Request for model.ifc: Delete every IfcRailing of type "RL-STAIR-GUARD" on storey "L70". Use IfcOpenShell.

First a look at what the model holds.

```python
import ifcopenshell
import ifcopenshell.util.element

model = ifcopenshell.open("model.ifc")
print(model.schema)
storey = next(s for s in model.by_type("IfcBuildingStorey") if s.Name == "L70")
railings = [e for e in ifcopenshell.util.element.get_decomposition(storey) if e.is_a("IfcRailing")]
seen = {}
for e in railings:
    element_type = ifcopenshell.util.element.get_type(e)
    name = element_type.Name if element_type not in (None, e) else None
    seen[name] = seen.get(name, 0) + 1
for name, count in sorted(seen.items(), key=str):
    print(count, "x", name)
```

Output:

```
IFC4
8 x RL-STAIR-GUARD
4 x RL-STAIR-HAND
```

```python
import ifcopenshell
import ifcopenshell.api.root
import ifcopenshell.util.element

model = ifcopenshell.open("model.ifc")

storey = next(s for s in model.by_type("IfcBuildingStorey") if s.Name == "L70")
railings = [e for e in ifcopenshell.util.element.get_decomposition(storey) if e.is_a("IfcRailing")]
targets = [e for e in railings if (t := ifcopenshell.util.element.get_type(e)) not in (None, e) and t.Name == "RL-STAIR-GUARD"]

for e in targets:
    ifcopenshell.api.root.remove_product(model, product=e)
print(len(targets), "removed")

model.write("model_edited.ifc")
```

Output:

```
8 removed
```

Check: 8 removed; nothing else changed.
